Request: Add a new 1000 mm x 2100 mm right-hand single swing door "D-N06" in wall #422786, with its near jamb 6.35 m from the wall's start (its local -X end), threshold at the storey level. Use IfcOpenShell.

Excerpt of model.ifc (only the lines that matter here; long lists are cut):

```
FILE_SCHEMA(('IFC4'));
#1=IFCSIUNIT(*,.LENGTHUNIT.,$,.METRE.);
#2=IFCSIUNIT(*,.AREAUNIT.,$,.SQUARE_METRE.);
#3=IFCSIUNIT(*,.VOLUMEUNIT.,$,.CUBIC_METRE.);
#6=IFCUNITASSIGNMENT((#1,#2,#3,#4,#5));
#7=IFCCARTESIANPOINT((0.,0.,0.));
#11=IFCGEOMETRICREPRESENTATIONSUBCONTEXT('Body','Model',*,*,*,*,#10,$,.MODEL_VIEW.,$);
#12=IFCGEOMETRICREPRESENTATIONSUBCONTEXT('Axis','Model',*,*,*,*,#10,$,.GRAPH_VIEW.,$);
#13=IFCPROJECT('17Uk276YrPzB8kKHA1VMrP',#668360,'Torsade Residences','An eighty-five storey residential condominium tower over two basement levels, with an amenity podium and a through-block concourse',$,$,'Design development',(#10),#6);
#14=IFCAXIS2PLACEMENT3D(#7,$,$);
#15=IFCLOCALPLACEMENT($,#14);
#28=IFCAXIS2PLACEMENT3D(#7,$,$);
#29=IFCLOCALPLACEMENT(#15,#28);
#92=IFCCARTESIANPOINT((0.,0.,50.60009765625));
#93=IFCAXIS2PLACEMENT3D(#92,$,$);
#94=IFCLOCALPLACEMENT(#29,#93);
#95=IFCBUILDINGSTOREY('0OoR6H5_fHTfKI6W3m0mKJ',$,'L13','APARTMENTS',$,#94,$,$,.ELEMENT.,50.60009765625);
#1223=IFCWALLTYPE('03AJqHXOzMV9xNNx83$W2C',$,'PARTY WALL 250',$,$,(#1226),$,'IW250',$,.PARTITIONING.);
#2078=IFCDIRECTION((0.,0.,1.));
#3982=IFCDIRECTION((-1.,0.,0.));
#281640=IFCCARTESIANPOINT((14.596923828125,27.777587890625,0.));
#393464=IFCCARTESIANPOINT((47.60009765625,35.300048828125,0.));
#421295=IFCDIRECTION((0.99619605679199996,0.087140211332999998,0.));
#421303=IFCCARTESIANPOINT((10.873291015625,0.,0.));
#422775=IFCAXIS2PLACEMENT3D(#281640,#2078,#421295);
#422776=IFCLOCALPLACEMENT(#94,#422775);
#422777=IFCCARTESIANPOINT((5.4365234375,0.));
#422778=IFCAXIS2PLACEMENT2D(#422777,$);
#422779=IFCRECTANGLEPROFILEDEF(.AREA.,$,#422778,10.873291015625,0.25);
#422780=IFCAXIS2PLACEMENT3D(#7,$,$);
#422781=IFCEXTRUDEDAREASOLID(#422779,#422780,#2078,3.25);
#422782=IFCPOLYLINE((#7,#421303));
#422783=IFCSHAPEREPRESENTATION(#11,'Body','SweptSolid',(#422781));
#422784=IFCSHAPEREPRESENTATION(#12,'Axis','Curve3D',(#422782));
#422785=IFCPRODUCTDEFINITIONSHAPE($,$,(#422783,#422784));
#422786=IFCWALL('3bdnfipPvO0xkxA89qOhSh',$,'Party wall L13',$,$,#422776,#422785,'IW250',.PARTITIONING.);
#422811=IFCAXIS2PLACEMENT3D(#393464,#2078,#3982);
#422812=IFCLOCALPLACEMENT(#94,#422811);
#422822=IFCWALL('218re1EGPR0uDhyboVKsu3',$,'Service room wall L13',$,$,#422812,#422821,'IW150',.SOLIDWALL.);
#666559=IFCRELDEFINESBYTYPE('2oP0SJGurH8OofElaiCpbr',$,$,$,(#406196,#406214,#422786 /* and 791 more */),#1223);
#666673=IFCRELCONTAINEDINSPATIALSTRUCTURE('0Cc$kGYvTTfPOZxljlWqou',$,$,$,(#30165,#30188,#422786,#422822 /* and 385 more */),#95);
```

```python
import numpy as np
import ifcopenshell
import ifcopenshell.api.feature
import ifcopenshell.api.geometry
import ifcopenshell.api.root
import ifcopenshell.api.spatial
import ifcopenshell.geom
import ifcopenshell.util.element
import ifcopenshell.util.placement
import ifcopenshell.util.representation
import ifcopenshell.util.shape
import ifcopenshell.util.unit

model = ifcopenshell.open("model.ifc")
unit_scale = ifcopenshell.util.unit.calculate_unit_scale(model)
settings = ifcopenshell.geom.settings()


def volume(element):
    """Net volume in cubic metres, openings subtracted."""
    shape = ifcopenshell.geom.create_shape(settings, element)
    return ifcopenshell.util.shape.get_volume(shape.geometry)


wall = model.by_guid("3bdnfipPvO0xkxA89qOhSh")
storey = ifcopenshell.util.element.get_container(wall, ifc_class="IfcBuildingStorey")
context = ifcopenshell.util.representation.get_context(model, "Model", "Body", "MODEL_VIEW")
before = volume(wall)

width, height, from_end, sill = 1, 2.1, 6.35, 0.0  # metres

# The wall runs along its own X axis, and the end named is its -X end.
wall_shape = ifcopenshell.geom.create_shape(settings, wall)
x, y, z = ifcopenshell.util.shape.get_vertices(wall_shape.geometry).T
start = x.min() + from_end
face, thickness = float(y.min()), float(y.max() - y.min())
wall_matrix = ifcopenshell.util.placement.get_local_placement(wall.ObjectPlacement)
level = ifcopenshell.util.placement.get_local_placement(storey.ObjectPlacement)[2, 3]


def in_wall(x, y):
    """Placement at x, y metres in the wall's axes, at sill height."""
    matrix = wall_matrix.copy()
    matrix[:, 3] = wall_matrix @ np.array([x / unit_scale, y / unit_scale, 0.0, 1.0])
    matrix[2, 3] = level + sill / unit_scale
    return matrix


# Opening: a box that overshoots both wall faces by 50 mm.
opening = ifcopenshell.api.root.create_entity(model, ifc_class="IfcOpeningElement", predefined_type="OPENING")
box = ifcopenshell.api.geometry.add_wall_representation(
    model, context=context, length=width, height=height, thickness=thickness + 0.1
)
ifcopenshell.api.geometry.assign_representation(model, product=opening, representation=box)
ifcopenshell.api.geometry.edit_object_placement(model, product=opening, matrix=in_wall(start, face - 0.05), is_si=False)
ifcopenshell.api.feature.add_feature(model, feature=opening, element=wall)

door = ifcopenshell.api.root.create_entity(model, ifc_class="IfcDoor", name="D-N06", predefined_type="DOOR")
door.OverallWidth, door.OverallHeight = width / unit_scale, height / unit_scale
door.OperationType = "SINGLE_SWING_RIGHT"
body = ifcopenshell.api.geometry.add_door_representation(
    model,
    context=context,
    overall_width=door.OverallWidth,
    overall_height=door.OverallHeight,
    operation_type="SINGLE_SWING_RIGHT",
    lining_properties={"LiningDepth": thickness / unit_scale, "ThresholdDepth": thickness / unit_scale},
)
ifcopenshell.api.geometry.assign_representation(model, product=door, representation=body)
ifcopenshell.api.spatial.assign_container(model, products=[door], relating_structure=storey)
ifcopenshell.api.feature.add_filling(model, opening=opening, element=door)

# The lining spans the wall, so the door starts at the wall face.
ifcopenshell.api.geometry.edit_object_placement(model, product=door, matrix=in_wall(start, face), is_si=False)

after = volume(wall)

print(f"wall volume {before:.3f} -> {after:.3f} m3")

model.write("model_updated.ifc")
```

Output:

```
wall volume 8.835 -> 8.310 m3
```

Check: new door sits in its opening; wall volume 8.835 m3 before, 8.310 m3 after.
